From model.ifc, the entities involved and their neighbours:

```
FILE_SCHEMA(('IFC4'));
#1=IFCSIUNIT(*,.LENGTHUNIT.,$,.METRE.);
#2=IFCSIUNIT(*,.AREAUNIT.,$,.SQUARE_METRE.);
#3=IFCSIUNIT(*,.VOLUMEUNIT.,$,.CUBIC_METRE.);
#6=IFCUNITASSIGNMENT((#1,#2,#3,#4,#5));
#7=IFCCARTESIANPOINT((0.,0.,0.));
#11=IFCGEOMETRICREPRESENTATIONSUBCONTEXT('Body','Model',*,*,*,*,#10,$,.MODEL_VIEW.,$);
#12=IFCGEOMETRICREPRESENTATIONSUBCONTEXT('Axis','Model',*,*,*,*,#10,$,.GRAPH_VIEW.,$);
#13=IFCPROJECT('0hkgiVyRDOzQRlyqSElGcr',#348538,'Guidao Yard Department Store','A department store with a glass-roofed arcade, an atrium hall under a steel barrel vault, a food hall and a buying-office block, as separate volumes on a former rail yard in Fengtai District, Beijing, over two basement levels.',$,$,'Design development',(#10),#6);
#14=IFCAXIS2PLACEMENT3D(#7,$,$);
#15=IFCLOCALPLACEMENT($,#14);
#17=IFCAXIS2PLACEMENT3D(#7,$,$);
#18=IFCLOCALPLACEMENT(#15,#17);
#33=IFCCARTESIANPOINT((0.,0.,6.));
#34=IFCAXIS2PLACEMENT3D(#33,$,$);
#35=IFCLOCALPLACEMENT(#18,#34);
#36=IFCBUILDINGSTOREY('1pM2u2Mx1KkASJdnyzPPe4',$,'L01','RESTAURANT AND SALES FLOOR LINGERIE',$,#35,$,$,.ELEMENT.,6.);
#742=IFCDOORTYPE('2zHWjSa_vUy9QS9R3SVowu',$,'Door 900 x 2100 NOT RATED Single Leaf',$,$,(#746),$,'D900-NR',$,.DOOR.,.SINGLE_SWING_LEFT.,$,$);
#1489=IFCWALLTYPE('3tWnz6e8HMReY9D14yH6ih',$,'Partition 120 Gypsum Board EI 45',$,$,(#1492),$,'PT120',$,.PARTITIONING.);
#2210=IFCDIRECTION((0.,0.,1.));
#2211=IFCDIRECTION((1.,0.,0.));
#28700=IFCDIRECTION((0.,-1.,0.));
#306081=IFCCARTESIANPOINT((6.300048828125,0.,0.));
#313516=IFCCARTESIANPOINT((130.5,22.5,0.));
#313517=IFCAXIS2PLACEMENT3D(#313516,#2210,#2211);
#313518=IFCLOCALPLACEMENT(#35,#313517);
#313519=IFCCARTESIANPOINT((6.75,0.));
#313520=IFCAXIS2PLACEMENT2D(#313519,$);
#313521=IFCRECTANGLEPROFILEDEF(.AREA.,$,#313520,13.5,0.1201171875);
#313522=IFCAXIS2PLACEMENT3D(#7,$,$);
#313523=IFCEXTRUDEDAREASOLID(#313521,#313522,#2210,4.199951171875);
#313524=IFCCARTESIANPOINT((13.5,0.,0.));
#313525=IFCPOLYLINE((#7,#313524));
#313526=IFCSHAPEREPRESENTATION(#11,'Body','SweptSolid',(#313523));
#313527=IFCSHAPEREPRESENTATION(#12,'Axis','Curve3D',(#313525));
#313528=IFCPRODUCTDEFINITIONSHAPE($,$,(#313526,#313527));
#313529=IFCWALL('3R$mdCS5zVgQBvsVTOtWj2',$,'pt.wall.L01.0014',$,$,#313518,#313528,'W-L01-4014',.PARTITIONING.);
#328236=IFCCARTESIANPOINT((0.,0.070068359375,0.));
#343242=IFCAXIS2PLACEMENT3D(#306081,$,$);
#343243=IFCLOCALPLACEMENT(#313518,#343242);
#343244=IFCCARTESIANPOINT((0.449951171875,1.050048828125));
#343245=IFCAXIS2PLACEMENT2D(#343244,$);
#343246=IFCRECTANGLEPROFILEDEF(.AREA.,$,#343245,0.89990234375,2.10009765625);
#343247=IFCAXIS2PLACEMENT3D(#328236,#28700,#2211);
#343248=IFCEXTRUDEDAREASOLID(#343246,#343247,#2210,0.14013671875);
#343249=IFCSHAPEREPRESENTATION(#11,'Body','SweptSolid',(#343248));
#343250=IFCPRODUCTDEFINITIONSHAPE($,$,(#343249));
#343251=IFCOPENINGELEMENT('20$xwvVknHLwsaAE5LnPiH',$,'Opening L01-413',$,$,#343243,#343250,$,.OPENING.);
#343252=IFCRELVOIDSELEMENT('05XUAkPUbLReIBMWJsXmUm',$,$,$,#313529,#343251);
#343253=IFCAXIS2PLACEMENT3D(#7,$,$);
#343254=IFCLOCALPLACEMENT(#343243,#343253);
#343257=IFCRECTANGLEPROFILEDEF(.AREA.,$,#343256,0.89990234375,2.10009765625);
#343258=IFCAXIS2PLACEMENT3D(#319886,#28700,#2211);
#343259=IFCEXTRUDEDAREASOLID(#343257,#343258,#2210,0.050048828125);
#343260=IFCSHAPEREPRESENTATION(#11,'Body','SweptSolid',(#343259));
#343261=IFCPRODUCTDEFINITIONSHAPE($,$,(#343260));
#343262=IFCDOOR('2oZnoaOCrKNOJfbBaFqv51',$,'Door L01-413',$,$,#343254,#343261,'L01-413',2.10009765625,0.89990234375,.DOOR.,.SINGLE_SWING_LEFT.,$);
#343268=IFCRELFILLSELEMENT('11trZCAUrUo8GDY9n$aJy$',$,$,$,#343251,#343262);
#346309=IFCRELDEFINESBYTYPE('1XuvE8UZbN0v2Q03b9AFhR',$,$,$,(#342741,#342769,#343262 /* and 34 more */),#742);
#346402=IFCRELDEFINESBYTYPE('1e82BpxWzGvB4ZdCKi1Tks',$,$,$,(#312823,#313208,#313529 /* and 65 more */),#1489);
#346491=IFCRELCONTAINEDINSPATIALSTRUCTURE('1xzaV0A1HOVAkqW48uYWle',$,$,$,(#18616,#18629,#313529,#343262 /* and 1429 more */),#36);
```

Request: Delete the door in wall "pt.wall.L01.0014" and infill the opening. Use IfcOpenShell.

```python
import ifcopenshell
import ifcopenshell.api.feature
import ifcopenshell.api.root
import ifcopenshell.geom
import ifcopenshell.util.shape

model = ifcopenshell.open("model.ifc")
settings = ifcopenshell.geom.settings()


def volume(element):
    """Net volume in cubic metres, openings subtracted."""
    shape = ifcopenshell.geom.create_shape(settings, element)
    return ifcopenshell.util.shape.get_volume(shape.geometry)


door = model.by_id(343262)
opening = door.FillsVoids[0].RelatingOpeningElement
wall = opening.VoidsElements[0].RelatingBuildingElement
before = volume(wall)

ifcopenshell.api.root.remove_product(model, product=door)
ifcopenshell.api.feature.remove_feature(model, feature=opening)

after = volume(wall)

print(f"wall volume {before:.3f} -> {after:.3f} m3")

model.write("model_rev.ifc")
```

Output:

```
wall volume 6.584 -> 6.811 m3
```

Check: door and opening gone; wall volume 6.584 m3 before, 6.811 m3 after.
